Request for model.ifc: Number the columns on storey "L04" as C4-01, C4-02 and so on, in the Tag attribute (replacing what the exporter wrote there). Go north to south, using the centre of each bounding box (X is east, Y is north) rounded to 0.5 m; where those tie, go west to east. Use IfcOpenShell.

First a look at what the model holds.

```python
import ifcopenshell
import ifcopenshell.util.element
import ifcopenshell.util.placement

model = ifcopenshell.open("model.ifc")
print(model.schema)
storey = next(s for s in model.by_type("IfcBuildingStorey") if s.Name == "L04")
columns = [e for e in ifcopenshell.util.element.get_decomposition(storey) if e.is_a("IfcColumn")]
for e in sorted(columns, key=lambda e: e.id()):
    origin = ifcopenshell.util.placement.get_local_placement(e.ObjectPlacement)[:3, 3]
    print(e.id(), e.Tag, e.Name, origin.round(2) + 0.0, sep=" | ")
```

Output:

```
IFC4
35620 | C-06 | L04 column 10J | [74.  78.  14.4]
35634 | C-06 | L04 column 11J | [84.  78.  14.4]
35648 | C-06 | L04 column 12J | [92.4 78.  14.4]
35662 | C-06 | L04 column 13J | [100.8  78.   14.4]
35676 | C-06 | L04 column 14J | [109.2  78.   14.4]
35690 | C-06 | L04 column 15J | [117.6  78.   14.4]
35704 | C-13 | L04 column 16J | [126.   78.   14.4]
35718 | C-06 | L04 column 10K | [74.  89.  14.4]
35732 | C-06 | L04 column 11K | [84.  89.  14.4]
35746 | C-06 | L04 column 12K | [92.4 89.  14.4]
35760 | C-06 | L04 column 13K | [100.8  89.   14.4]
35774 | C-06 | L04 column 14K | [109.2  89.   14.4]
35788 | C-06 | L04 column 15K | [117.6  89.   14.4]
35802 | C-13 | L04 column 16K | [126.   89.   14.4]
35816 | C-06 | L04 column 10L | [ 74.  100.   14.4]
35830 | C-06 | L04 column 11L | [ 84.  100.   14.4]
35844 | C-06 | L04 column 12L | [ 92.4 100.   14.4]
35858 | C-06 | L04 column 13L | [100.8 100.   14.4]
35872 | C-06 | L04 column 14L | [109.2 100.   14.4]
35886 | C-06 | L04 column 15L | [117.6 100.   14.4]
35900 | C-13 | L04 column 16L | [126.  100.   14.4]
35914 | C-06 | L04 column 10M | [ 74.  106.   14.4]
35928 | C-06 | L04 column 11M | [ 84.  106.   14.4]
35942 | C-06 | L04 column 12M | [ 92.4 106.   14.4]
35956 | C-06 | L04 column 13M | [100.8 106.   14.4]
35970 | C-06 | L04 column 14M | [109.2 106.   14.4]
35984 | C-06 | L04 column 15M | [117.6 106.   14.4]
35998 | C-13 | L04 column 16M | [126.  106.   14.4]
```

```python
import ifcopenshell
import ifcopenshell.geom
import ifcopenshell.util.element
import ifcopenshell.util.shape

model = ifcopenshell.open("model.ifc")
settings = ifcopenshell.geom.settings()
settings.set("use-world-coords", True)


def centre(element):
    shape = ifcopenshell.geom.create_shape(settings, element)
    return ifcopenshell.util.shape.get_bbox_centroid(shape.geometry)


storey = next(s for s in model.by_type("IfcBuildingStorey") if s.Name == "L04")
columns = [e for e in ifcopenshell.util.element.get_decomposition(storey) if e.is_a("IfcColumn")]

# Insertion points can sit at a corner or the storey origin, so sort by the geometry (in metres).
centres = {e: centre(e) for e in columns}
columns.sort(key=lambda e: (-round(centres[e][1] / 0.5), centres[e][0]))

for i, e in enumerate(columns, start=1):
    number = f"C4-{i:02d}"
    e.Tag = number
    print(e.id(), number)

model.write("model-out.ifc")
```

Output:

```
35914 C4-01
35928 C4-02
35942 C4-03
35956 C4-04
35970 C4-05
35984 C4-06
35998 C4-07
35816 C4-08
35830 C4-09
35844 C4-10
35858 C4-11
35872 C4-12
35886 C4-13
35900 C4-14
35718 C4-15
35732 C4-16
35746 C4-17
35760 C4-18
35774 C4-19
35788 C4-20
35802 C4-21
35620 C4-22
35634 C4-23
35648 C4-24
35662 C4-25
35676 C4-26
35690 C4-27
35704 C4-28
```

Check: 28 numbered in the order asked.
